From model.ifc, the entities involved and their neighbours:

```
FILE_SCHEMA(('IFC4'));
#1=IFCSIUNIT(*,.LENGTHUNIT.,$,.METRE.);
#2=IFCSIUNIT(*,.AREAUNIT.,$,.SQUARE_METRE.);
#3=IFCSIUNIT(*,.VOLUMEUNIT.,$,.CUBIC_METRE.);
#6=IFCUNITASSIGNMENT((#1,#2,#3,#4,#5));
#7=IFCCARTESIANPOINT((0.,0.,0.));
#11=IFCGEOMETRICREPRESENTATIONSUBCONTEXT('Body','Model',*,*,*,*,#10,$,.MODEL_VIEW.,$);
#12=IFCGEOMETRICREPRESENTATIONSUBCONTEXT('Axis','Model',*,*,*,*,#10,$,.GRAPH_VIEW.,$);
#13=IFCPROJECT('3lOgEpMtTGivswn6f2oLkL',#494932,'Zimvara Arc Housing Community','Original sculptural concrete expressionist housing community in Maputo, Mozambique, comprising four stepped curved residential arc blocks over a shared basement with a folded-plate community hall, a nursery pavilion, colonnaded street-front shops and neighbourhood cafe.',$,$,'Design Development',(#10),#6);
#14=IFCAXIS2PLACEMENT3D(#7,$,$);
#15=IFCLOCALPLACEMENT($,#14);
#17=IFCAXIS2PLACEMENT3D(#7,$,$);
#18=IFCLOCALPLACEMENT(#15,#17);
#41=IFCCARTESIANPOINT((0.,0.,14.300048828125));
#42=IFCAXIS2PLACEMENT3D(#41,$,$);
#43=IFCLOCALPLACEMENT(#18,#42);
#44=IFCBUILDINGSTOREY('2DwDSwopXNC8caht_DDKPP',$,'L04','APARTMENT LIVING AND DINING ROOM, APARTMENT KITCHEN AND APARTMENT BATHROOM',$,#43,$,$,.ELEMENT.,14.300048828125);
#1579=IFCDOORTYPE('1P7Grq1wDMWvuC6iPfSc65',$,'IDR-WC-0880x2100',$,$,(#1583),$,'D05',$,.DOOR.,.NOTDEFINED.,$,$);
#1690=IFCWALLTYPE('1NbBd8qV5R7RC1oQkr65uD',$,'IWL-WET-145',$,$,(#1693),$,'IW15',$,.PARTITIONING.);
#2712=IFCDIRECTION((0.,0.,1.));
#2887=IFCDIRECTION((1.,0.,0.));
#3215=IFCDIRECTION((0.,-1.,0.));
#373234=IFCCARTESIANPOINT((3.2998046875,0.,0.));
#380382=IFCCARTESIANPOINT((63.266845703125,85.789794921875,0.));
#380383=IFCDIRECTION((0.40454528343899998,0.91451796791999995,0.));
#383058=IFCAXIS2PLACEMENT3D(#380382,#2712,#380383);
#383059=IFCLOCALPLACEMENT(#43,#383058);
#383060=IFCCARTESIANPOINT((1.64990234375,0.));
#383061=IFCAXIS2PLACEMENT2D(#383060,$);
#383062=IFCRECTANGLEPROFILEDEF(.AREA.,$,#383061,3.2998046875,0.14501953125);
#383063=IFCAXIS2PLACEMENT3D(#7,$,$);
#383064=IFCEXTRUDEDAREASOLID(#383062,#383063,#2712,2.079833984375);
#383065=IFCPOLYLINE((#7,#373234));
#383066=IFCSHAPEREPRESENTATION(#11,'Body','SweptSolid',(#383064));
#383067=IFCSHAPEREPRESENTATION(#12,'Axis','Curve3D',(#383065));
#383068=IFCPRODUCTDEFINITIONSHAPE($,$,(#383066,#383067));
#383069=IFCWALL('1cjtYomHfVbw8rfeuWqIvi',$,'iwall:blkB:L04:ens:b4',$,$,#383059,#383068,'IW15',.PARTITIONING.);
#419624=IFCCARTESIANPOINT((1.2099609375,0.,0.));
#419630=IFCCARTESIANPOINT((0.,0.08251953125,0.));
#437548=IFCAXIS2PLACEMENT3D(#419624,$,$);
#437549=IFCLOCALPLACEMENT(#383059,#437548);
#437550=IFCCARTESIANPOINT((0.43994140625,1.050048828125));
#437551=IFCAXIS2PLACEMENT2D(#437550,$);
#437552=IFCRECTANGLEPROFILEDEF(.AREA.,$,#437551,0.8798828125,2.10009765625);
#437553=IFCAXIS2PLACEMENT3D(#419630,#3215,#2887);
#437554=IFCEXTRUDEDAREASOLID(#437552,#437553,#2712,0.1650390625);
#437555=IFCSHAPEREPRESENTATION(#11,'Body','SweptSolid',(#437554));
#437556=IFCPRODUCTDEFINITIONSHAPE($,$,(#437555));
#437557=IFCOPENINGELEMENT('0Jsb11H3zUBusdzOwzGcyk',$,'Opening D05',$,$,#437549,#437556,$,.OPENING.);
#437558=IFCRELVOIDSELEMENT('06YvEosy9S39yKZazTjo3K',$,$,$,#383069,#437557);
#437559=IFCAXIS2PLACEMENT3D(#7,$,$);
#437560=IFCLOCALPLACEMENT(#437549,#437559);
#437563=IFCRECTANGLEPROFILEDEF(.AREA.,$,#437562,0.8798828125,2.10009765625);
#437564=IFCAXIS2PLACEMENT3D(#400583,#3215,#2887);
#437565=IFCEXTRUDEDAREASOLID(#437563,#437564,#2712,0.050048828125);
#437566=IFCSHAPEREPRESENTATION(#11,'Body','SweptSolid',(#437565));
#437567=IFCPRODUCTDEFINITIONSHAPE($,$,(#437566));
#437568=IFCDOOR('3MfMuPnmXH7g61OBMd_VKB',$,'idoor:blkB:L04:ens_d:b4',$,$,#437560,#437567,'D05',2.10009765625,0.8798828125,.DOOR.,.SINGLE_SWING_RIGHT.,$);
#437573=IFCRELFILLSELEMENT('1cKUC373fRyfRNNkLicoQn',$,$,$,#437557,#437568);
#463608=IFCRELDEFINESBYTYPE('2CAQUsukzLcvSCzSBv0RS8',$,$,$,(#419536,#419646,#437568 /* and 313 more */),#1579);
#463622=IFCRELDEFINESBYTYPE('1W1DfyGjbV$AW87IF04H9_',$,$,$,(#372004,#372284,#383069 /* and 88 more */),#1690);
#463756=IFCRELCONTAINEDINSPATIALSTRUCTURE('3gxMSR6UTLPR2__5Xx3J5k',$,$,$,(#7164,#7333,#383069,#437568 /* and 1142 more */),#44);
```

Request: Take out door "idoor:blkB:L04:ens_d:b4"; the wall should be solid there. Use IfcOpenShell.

```python
import ifcopenshell
import ifcopenshell.api.feature
import ifcopenshell.api.root
import ifcopenshell.geom
import ifcopenshell.util.shape

model = ifcopenshell.open("model.ifc")
settings = ifcopenshell.geom.settings()


def volume(element):
    """Net volume in cubic metres, openings subtracted."""
    shape = ifcopenshell.geom.create_shape(settings, element)
    return ifcopenshell.util.shape.get_volume(shape.geometry)


door = model.by_id(437568)
opening = door.FillsVoids[0].RelatingOpeningElement
wall = opening.VoidsElements[0].RelatingBuildingElement
before = volume(wall)

ifcopenshell.api.root.remove_product(model, product=door)
ifcopenshell.api.feature.remove_feature(model, feature=opening)

after = volume(wall)

print(f"wall volume {before:.3f} -> {after:.3f} m3")

model.write("model_updated.ifc")
```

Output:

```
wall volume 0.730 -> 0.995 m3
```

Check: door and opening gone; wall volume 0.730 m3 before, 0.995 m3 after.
